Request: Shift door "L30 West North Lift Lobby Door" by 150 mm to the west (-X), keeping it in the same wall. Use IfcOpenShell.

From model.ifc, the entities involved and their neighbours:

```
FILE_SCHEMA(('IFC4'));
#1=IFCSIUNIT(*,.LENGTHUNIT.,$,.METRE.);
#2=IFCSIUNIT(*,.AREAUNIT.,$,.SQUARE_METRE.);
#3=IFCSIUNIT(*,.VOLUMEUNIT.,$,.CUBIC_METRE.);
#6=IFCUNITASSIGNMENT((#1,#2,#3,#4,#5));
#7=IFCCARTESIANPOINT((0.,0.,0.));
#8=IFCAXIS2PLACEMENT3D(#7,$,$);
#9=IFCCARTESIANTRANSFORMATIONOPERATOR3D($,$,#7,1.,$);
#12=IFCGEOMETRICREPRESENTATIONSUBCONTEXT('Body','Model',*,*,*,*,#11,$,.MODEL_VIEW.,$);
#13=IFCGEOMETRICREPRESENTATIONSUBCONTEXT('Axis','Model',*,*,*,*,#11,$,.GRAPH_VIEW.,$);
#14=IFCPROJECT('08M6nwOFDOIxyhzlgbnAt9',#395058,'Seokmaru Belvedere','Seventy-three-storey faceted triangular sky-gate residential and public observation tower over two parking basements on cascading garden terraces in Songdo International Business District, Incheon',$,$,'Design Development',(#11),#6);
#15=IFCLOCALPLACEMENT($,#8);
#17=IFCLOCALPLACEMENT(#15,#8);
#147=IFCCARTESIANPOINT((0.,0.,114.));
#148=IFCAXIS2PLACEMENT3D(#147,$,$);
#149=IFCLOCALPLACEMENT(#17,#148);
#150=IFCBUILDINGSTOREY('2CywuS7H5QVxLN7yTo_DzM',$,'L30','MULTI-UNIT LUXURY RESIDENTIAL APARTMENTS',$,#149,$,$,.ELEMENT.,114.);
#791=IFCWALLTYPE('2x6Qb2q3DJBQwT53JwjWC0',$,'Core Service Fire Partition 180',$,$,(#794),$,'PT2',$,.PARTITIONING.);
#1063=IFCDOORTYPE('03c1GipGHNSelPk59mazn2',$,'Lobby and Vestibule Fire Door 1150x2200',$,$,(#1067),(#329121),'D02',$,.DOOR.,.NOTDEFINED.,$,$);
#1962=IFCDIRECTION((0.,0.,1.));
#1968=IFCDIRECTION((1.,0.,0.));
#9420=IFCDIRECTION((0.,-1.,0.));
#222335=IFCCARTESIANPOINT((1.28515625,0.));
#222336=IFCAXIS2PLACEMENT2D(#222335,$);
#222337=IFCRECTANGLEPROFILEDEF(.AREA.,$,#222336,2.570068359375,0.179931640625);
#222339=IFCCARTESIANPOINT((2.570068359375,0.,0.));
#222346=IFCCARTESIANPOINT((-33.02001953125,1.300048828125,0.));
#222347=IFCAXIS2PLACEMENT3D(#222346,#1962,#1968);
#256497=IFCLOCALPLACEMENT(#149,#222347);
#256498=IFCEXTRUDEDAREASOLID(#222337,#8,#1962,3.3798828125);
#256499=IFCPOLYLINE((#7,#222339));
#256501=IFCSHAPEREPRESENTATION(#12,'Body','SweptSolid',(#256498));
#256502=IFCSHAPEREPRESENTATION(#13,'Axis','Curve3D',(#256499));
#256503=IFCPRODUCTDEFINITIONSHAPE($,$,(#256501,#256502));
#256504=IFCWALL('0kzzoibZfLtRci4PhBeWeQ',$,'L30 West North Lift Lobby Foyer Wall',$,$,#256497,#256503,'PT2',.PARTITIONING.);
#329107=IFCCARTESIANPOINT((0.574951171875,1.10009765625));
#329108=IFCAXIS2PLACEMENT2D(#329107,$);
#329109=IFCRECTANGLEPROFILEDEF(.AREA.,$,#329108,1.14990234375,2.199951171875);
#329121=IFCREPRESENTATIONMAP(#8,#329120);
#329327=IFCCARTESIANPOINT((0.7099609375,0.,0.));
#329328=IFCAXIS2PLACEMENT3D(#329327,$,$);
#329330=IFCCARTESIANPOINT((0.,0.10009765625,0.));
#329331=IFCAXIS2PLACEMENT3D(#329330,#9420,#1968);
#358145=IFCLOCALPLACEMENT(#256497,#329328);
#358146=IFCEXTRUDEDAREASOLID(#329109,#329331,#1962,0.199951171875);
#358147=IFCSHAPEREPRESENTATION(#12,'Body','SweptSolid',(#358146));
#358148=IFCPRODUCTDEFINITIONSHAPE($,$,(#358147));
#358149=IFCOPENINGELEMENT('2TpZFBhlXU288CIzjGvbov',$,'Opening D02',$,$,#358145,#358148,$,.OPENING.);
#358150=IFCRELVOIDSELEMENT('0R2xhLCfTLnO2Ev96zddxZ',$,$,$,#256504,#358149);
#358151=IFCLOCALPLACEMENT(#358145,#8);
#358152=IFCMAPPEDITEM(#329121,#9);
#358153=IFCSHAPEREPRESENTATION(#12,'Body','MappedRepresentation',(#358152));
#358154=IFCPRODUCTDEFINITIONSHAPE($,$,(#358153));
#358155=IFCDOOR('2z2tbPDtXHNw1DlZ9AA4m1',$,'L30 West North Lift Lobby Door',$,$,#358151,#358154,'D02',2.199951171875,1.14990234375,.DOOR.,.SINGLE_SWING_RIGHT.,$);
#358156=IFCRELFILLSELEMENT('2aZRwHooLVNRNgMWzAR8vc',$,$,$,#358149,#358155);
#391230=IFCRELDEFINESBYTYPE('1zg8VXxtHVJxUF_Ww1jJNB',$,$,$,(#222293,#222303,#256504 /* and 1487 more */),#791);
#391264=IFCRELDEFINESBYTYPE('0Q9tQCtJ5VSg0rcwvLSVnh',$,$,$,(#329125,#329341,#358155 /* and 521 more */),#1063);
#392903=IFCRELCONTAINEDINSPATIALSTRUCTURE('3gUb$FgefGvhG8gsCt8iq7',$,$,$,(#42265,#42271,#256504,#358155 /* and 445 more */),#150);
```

```python
import ifcopenshell
import ifcopenshell.api.geometry
import ifcopenshell.util.placement
import ifcopenshell.util.unit

model = ifcopenshell.open("model.ifc")
unit_scale = ifcopenshell.util.unit.calculate_unit_scale(model)

door = model.by_id(358155)
opening = door.FillsVoids[0].RelatingOpeningElement
wall = opening.VoidsElements[0].RelatingBuildingElement

wall_matrix = ifcopenshell.util.placement.get_local_placement(wall.ObjectPlacement)
shift = wall_matrix[:3, 0] * -0.15 / unit_scale
before = ifcopenshell.util.placement.get_local_placement(door.ObjectPlacement)[:3, 3].copy()

# The door is placed relative to its opening, so it follows when the opening moves.
matrix = ifcopenshell.util.placement.get_local_placement(opening.ObjectPlacement)
matrix[:3, 3] += shift
ifcopenshell.api.geometry.edit_object_placement(
    model, product=opening, matrix=matrix, is_si=False, should_transform_children=True
)

after = ifcopenshell.util.placement.get_local_placement(door.ObjectPlacement)[:3, 3]
print("door moved by", (after - before).round(3) + 0.0)

model.write("model-out.ifc")
```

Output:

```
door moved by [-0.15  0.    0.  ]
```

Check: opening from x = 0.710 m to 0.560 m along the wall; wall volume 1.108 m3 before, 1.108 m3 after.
